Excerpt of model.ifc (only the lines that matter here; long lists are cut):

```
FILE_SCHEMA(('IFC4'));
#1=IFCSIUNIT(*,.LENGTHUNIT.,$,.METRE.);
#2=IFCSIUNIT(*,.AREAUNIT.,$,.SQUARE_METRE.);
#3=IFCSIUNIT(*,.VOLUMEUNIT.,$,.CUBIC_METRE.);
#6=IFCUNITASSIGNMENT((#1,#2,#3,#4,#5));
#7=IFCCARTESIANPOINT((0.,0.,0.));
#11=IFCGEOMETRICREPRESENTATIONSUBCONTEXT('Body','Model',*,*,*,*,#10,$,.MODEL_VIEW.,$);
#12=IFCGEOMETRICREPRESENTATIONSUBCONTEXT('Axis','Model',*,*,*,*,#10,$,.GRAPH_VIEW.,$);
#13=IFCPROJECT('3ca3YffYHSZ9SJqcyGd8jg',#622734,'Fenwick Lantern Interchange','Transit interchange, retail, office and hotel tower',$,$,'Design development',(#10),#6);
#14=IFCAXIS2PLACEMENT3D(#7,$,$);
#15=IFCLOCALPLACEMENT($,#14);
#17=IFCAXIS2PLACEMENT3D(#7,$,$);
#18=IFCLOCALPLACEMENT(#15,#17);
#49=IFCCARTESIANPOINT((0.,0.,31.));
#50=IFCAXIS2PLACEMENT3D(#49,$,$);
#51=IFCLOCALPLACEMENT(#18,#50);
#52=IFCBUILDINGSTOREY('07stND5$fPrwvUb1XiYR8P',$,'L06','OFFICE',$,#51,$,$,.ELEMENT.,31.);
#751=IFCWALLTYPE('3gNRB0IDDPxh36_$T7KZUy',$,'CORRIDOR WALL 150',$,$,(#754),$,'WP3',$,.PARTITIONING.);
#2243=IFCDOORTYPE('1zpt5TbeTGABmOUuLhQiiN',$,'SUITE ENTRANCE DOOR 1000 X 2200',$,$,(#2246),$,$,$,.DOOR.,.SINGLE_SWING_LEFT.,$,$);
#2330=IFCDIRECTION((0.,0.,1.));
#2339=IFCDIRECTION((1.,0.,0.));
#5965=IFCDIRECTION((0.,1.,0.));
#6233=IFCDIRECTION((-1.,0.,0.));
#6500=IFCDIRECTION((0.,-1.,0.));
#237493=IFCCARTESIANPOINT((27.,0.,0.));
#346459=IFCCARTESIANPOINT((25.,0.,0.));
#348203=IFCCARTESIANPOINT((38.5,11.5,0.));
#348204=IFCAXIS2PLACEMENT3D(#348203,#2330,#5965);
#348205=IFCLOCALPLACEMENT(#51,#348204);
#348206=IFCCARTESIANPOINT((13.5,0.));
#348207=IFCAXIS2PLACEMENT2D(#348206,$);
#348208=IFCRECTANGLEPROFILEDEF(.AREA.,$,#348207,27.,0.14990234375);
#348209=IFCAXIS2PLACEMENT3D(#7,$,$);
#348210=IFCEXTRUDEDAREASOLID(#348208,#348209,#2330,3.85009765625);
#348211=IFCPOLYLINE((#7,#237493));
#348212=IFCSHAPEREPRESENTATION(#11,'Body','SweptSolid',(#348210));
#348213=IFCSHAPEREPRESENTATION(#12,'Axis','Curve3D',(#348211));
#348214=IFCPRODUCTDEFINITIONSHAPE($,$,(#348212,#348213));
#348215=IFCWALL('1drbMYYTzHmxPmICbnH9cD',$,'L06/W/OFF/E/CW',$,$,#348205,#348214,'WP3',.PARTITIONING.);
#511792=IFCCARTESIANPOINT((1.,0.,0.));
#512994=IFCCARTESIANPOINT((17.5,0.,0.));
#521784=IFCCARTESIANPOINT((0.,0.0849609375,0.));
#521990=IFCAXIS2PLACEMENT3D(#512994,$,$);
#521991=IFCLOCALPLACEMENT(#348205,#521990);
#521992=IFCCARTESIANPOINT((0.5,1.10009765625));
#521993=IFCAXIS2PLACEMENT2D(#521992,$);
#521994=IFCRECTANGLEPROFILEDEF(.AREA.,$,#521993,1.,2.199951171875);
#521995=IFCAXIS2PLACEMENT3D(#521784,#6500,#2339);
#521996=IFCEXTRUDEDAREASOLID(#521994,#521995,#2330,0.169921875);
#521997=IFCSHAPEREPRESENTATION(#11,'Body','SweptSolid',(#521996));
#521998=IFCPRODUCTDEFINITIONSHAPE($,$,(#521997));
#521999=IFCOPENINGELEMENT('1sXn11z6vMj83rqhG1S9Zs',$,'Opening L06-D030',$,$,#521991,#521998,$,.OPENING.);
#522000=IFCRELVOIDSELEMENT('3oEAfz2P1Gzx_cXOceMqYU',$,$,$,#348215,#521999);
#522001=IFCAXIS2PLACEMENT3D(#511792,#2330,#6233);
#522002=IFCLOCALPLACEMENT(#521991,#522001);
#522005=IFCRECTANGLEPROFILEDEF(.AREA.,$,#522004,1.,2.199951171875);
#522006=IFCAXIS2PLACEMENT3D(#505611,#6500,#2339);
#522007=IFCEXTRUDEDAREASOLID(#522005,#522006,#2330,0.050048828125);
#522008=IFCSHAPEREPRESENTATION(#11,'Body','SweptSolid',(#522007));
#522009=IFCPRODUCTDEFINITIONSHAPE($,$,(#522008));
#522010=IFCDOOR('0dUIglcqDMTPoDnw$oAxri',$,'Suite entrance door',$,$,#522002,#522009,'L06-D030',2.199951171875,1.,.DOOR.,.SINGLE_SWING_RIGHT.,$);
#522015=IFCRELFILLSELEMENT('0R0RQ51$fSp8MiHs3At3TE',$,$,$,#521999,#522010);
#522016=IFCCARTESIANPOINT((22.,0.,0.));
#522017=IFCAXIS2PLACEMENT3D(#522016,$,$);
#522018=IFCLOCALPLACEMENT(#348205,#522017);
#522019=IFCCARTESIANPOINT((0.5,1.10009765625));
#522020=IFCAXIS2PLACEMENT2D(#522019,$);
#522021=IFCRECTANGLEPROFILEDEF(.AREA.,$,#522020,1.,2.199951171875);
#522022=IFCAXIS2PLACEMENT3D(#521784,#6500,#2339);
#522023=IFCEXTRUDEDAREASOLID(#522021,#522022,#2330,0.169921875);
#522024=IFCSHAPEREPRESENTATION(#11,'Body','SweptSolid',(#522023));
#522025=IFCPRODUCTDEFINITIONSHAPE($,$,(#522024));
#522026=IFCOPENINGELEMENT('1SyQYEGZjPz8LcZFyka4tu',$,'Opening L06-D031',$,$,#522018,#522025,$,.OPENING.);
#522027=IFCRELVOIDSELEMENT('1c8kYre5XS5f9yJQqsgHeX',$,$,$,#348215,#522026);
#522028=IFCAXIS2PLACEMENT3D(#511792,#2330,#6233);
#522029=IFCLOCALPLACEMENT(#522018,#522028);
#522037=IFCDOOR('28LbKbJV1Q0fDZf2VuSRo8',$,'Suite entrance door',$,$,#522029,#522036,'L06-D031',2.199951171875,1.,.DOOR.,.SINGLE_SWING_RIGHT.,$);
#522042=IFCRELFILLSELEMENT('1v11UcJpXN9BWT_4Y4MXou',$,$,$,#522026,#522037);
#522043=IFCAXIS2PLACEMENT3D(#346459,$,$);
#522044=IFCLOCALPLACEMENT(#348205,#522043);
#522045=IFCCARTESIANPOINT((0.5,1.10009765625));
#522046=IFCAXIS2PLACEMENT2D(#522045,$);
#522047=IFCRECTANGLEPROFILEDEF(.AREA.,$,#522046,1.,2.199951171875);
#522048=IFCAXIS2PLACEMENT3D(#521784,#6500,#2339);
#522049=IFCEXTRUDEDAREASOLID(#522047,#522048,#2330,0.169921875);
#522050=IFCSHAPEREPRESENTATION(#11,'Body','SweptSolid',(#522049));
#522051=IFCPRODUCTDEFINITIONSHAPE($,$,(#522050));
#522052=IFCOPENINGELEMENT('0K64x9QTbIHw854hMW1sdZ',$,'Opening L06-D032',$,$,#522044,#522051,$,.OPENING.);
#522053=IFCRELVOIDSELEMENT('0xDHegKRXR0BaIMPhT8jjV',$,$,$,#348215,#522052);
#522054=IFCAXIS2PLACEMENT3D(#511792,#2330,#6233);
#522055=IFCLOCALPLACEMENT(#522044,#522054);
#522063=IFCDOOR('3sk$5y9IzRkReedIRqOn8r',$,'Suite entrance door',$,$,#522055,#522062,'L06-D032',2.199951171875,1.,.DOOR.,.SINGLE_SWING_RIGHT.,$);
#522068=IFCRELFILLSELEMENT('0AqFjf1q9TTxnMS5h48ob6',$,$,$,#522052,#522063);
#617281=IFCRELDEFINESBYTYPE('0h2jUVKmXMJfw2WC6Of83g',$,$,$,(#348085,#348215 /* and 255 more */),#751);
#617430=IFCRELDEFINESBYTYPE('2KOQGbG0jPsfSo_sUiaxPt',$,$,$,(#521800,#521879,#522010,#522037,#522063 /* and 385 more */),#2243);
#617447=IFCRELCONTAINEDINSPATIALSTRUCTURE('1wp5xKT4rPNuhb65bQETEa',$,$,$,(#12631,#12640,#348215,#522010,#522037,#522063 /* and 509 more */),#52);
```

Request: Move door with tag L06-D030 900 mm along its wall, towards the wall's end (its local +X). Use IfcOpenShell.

```python
import ifcopenshell
import ifcopenshell.api.geometry
import ifcopenshell.util.placement
import ifcopenshell.util.unit

model = ifcopenshell.open("model.ifc")
unit_scale = ifcopenshell.util.unit.calculate_unit_scale(model)

door = model.by_guid("0dUIglcqDMTPoDnw$oAxri")
opening = door.FillsVoids[0].RelatingOpeningElement
wall = opening.VoidsElements[0].RelatingBuildingElement

wall_matrix = ifcopenshell.util.placement.get_local_placement(wall.ObjectPlacement)
shift = wall_matrix[:3, 0] * 0.9 / unit_scale
before = ifcopenshell.util.placement.get_local_placement(door.ObjectPlacement)[:3, 3].copy()

# The door is placed relative to its opening, so it follows when the opening moves.
matrix = ifcopenshell.util.placement.get_local_placement(opening.ObjectPlacement)
matrix[:3, 3] += shift
ifcopenshell.api.geometry.edit_object_placement(
    model, product=opening, matrix=matrix, is_si=False, should_transform_children=True
)

after = ifcopenshell.util.placement.get_local_placement(door.ObjectPlacement)[:3, 3]
print("door moved by", (after - before).round(3) + 0.0)

model.write("model_updated.ifc")
```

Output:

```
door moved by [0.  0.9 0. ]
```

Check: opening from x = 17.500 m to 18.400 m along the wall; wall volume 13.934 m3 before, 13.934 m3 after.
